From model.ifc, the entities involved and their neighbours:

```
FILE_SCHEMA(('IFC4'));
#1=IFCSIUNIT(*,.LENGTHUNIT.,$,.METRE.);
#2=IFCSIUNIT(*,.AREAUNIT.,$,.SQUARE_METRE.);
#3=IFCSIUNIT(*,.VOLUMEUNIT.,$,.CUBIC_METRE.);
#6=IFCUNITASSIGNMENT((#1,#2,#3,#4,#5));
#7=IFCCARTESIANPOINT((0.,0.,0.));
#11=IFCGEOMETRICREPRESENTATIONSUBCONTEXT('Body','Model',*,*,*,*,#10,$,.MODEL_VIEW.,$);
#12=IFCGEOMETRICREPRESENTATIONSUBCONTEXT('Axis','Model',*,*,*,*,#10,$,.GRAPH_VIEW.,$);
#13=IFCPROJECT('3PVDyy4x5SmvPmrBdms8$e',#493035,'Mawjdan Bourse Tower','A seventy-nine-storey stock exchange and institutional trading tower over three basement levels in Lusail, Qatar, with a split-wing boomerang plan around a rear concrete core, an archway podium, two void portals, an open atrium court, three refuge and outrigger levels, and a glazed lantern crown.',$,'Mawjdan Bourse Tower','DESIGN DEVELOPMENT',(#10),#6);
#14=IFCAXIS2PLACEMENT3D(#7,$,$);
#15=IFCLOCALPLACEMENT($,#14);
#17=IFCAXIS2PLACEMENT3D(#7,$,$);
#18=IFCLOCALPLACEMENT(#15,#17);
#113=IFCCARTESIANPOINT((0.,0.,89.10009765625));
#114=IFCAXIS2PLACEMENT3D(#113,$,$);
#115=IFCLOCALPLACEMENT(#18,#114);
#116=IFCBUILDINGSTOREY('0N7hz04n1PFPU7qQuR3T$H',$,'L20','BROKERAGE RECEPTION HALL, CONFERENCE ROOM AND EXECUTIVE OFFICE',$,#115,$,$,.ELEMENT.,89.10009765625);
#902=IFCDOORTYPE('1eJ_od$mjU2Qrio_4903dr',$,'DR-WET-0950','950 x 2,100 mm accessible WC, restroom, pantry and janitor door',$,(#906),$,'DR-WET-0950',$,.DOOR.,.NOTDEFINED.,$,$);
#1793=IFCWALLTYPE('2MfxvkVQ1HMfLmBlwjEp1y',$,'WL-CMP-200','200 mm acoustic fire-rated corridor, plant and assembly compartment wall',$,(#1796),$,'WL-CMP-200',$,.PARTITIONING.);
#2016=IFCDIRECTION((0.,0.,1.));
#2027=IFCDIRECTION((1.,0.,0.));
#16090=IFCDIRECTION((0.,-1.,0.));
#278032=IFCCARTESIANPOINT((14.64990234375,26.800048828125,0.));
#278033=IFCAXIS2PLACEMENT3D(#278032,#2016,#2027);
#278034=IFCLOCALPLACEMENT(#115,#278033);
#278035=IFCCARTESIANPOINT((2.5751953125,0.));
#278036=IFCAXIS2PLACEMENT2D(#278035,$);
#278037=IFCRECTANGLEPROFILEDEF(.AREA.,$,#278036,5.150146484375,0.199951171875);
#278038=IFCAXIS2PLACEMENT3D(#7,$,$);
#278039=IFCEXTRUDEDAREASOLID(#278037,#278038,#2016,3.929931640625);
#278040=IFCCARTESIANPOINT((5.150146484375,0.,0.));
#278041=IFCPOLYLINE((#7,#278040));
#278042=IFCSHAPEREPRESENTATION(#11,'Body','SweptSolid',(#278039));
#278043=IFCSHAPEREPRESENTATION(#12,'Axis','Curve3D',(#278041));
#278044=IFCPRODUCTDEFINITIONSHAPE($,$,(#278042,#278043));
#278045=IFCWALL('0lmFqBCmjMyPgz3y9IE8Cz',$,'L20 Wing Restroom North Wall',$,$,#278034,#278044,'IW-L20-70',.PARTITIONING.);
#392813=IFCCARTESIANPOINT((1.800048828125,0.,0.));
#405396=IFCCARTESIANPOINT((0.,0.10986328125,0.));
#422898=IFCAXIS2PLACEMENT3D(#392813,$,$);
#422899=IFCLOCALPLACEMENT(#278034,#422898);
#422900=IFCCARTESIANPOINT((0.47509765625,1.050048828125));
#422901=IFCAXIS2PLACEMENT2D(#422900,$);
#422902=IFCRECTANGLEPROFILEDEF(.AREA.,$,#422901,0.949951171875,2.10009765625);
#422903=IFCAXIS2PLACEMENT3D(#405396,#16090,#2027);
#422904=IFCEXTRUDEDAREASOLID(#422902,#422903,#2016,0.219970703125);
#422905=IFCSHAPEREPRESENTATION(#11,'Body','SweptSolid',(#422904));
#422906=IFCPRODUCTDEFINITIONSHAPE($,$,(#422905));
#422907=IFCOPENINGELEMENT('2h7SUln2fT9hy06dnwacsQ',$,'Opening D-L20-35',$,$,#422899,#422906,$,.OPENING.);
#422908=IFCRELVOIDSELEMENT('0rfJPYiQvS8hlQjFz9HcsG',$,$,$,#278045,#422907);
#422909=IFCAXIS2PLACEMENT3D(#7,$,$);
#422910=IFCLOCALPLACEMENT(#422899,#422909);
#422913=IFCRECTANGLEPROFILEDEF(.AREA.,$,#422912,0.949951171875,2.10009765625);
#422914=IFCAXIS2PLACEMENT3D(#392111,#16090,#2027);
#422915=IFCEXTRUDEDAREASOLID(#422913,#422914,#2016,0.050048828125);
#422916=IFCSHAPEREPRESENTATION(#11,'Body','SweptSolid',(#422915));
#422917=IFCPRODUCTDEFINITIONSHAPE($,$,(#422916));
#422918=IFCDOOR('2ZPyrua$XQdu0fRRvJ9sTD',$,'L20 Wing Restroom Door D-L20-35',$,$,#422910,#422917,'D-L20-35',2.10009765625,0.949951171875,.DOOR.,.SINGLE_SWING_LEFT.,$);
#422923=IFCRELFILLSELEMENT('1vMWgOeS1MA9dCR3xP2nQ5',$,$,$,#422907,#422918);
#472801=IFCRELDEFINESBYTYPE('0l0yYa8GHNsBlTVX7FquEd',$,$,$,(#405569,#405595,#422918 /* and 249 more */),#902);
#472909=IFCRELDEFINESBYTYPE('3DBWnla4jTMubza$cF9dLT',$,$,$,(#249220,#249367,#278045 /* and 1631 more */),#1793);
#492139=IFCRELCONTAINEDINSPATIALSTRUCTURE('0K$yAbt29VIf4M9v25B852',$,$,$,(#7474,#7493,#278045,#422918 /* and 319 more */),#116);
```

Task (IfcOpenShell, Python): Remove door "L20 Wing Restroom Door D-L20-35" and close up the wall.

```python
import ifcopenshell
import ifcopenshell.api.feature
import ifcopenshell.api.root
import ifcopenshell.geom
import ifcopenshell.util.shape

model = ifcopenshell.open("model.ifc")
settings = ifcopenshell.geom.settings()


def volume(element):
    """Net volume in cubic metres, openings subtracted."""
    shape = ifcopenshell.geom.create_shape(settings, element)
    return ifcopenshell.util.shape.get_volume(shape.geometry)


door = model.by_id(422918)
opening = door.FillsVoids[0].RelatingOpeningElement
wall = opening.VoidsElements[0].RelatingBuildingElement
before = volume(wall)

ifcopenshell.api.root.remove_product(model, product=door)
ifcopenshell.api.feature.remove_feature(model, feature=opening)

after = volume(wall)

print(f"wall volume {before:.3f} -> {after:.3f} m3")

model.write("model_edited.ifc")
```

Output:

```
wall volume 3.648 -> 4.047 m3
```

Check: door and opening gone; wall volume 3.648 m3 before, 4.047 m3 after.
